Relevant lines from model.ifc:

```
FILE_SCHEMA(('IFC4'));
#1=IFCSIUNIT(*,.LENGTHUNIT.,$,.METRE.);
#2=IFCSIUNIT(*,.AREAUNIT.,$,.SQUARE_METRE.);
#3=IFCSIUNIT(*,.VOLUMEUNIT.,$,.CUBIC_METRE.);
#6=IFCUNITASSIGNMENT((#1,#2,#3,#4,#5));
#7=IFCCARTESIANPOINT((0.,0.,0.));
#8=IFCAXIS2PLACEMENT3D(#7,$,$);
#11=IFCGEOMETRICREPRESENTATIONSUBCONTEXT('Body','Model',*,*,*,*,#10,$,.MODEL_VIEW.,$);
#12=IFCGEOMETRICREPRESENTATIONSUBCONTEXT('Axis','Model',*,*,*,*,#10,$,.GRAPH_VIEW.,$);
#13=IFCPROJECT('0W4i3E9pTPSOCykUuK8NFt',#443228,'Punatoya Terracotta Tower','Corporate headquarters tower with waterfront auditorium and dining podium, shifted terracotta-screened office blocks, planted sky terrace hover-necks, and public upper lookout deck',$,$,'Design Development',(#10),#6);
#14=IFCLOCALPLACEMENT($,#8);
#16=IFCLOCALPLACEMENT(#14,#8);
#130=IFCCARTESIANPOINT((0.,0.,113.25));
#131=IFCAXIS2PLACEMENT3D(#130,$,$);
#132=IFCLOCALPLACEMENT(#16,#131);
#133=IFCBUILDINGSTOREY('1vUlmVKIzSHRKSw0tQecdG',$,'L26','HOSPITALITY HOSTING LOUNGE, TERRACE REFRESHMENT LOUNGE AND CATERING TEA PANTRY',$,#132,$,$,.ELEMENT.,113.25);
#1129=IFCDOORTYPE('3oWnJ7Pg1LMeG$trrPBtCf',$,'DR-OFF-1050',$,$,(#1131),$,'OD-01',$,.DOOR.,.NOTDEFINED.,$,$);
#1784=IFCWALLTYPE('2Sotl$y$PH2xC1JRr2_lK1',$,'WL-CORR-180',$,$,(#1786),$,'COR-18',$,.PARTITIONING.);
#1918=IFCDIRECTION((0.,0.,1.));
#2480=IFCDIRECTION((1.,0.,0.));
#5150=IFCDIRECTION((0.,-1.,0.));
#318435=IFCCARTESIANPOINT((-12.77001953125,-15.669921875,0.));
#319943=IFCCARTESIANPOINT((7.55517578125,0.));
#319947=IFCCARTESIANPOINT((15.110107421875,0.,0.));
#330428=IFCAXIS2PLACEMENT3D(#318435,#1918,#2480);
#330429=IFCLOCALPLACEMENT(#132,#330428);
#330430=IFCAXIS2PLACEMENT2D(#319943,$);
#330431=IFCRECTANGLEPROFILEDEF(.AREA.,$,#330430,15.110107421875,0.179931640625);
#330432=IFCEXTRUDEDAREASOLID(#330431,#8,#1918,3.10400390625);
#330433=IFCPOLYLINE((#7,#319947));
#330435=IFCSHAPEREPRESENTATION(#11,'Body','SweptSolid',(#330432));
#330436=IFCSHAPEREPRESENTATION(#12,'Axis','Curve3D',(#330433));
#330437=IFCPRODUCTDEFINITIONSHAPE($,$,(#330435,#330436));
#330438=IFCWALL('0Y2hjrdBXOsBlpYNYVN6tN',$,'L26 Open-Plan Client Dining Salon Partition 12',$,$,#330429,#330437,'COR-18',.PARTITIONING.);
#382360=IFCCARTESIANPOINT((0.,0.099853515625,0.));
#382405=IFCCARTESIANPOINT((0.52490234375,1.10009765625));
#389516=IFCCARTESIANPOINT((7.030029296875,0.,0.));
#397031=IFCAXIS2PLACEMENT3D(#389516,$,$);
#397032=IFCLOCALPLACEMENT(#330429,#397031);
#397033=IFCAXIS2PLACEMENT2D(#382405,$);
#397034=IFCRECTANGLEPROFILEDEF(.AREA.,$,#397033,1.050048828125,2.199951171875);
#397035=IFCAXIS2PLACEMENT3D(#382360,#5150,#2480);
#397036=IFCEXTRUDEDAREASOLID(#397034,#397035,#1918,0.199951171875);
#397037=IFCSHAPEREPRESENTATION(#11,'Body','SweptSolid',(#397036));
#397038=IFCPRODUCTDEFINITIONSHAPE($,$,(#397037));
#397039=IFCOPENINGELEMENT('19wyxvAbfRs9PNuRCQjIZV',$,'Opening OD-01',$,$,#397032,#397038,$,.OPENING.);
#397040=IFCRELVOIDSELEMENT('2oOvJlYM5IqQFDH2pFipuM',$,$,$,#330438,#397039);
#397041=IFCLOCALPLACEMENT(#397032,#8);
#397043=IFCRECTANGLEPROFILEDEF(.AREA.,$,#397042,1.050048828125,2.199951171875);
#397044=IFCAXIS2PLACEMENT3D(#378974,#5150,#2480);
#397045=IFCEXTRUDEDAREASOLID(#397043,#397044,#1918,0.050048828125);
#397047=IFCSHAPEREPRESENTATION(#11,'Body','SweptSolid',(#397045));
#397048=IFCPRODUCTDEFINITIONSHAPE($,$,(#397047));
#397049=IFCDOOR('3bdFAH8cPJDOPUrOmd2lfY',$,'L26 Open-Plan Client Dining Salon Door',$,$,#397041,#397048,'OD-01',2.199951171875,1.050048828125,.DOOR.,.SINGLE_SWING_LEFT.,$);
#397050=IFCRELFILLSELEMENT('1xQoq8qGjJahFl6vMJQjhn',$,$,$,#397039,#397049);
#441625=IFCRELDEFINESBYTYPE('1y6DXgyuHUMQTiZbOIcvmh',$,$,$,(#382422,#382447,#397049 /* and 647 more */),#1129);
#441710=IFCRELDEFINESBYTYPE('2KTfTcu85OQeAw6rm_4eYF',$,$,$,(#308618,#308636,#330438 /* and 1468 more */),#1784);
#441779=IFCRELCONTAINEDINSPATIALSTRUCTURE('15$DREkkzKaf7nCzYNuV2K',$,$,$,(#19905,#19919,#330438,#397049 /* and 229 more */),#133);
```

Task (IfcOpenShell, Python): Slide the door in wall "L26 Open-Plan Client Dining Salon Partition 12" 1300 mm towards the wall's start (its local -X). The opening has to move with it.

```python
import ifcopenshell
import ifcopenshell.api.geometry
import ifcopenshell.util.placement
import ifcopenshell.util.unit

model = ifcopenshell.open("model.ifc")
unit_scale = ifcopenshell.util.unit.calculate_unit_scale(model)

door = model.by_guid("3bdFAH8cPJDOPUrOmd2lfY")
opening = door.FillsVoids[0].RelatingOpeningElement
wall = opening.VoidsElements[0].RelatingBuildingElement

wall_matrix = ifcopenshell.util.placement.get_local_placement(wall.ObjectPlacement)
shift = wall_matrix[:3, 0] * -1.3 / unit_scale
before = ifcopenshell.util.placement.get_local_placement(door.ObjectPlacement)[:3, 3].copy()

# The door is placed relative to its opening, so it follows when the opening moves.
matrix = ifcopenshell.util.placement.get_local_placement(opening.ObjectPlacement)
matrix[:3, 3] += shift
ifcopenshell.api.geometry.edit_object_placement(
    model, product=opening, matrix=matrix, is_si=False, should_transform_children=True
)

after = ifcopenshell.util.placement.get_local_placement(door.ObjectPlacement)[:3, 3]
print("door moved by", (after - before).round(3) + 0.0)

model.write("model-out.ifc")
```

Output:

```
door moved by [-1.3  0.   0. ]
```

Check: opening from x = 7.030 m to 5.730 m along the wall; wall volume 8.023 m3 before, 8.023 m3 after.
